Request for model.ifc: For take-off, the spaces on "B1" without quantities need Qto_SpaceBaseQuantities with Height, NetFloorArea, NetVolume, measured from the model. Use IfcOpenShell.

First a look at what the model holds.

```python
import ifcopenshell
import ifcopenshell.util.element
import ifcopenshell.util.unit

model = ifcopenshell.open("model.ifc")
print(model.schema)
for unit_type in ("LENGTHUNIT", "AREAUNIT", "VOLUMEUNIT"):
    print(unit_type, ifcopenshell.util.unit.calculate_unit_scale(model, unit_type))
storey = next(s for s in model.by_type("IfcBuildingStorey") if s.Name == "B1")
spaces = [e for e in ifcopenshell.util.element.get_decomposition(storey) if e.is_a("IfcSpace")]
for e in sorted(spaces, key=lambda e: e.id()):
    print(e.id(), e.is_a(), e.Name, list(ifcopenshell.util.element.get_psets(e, qtos_only=True)), sep=" | ")
```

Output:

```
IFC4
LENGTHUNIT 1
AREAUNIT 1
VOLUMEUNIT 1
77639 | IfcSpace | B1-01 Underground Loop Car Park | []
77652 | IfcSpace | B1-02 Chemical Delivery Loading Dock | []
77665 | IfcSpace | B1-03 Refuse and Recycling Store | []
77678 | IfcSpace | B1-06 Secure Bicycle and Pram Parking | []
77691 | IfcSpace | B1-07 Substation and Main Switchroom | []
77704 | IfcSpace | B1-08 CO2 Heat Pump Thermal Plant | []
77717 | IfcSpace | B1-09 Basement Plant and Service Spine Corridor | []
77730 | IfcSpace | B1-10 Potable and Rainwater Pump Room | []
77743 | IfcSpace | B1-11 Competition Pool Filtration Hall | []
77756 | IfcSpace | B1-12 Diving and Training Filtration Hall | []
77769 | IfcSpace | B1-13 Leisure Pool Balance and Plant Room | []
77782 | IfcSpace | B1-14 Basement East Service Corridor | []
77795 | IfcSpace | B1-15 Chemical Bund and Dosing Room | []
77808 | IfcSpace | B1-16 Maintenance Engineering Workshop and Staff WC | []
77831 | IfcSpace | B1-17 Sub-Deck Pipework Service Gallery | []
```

```python
import ifcopenshell
import ifcopenshell.api.pset
import ifcopenshell.geom
import ifcopenshell.util.element
import ifcopenshell.util.shape
import ifcopenshell.util.unit

model = ifcopenshell.open("model.ifc")
unit_scale = ifcopenshell.util.unit.calculate_unit_scale(model)
area_scale = ifcopenshell.util.unit.calculate_unit_scale(model, "AREAUNIT")
volume_scale = ifcopenshell.util.unit.calculate_unit_scale(model, "VOLUMEUNIT")
settings = ifcopenshell.geom.settings()

storey = next(s for s in model.by_type("IfcBuildingStorey") if s.Name == "B1")
spaces = [e for e in ifcopenshell.util.element.get_decomposition(storey) if e.is_a("IfcSpace")]

for e in sorted(spaces, key=lambda e: e.id()):
    if ifcopenshell.util.element.get_psets(e, qtos_only=True, should_inherit=False):
        continue
    # Geometry comes back in metres, in the element's own axes.
    shape = ifcopenshell.geom.create_shape(settings, e)
    values = {
        "Height": ifcopenshell.util.shape.get_z(shape.geometry) / unit_scale,
        "NetFloorArea": ifcopenshell.util.shape.get_footprint_area(shape.geometry) / area_scale,
        "NetVolume": ifcopenshell.util.shape.get_volume(shape.geometry) / volume_scale,
    }
    qto = ifcopenshell.api.pset.add_qto(model, product=e, name="Qto_SpaceBaseQuantities")
    ifcopenshell.api.pset.edit_qto(model, qto=qto, properties=values)
    print(e.id(), {k: round(v, 3) for k, v in values.items()})

model.write("model_updated.ifc")
```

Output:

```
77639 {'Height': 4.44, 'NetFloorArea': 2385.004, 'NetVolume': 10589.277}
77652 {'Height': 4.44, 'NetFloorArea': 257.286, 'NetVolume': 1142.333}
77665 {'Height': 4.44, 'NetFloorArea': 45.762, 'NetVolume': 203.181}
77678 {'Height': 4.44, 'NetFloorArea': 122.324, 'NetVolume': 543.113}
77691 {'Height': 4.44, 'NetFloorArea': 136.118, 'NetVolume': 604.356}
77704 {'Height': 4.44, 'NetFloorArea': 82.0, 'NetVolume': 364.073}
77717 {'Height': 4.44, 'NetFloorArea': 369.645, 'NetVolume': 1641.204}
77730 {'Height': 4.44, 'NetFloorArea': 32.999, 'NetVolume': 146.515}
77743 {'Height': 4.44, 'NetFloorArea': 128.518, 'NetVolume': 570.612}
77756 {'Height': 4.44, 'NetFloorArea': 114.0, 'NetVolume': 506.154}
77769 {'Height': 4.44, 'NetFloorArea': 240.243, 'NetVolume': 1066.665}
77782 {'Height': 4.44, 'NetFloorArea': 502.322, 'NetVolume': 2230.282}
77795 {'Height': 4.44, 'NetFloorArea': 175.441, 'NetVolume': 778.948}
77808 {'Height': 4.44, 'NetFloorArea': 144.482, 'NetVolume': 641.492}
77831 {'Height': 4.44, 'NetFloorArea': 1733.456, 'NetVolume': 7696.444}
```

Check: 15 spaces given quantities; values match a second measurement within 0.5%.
